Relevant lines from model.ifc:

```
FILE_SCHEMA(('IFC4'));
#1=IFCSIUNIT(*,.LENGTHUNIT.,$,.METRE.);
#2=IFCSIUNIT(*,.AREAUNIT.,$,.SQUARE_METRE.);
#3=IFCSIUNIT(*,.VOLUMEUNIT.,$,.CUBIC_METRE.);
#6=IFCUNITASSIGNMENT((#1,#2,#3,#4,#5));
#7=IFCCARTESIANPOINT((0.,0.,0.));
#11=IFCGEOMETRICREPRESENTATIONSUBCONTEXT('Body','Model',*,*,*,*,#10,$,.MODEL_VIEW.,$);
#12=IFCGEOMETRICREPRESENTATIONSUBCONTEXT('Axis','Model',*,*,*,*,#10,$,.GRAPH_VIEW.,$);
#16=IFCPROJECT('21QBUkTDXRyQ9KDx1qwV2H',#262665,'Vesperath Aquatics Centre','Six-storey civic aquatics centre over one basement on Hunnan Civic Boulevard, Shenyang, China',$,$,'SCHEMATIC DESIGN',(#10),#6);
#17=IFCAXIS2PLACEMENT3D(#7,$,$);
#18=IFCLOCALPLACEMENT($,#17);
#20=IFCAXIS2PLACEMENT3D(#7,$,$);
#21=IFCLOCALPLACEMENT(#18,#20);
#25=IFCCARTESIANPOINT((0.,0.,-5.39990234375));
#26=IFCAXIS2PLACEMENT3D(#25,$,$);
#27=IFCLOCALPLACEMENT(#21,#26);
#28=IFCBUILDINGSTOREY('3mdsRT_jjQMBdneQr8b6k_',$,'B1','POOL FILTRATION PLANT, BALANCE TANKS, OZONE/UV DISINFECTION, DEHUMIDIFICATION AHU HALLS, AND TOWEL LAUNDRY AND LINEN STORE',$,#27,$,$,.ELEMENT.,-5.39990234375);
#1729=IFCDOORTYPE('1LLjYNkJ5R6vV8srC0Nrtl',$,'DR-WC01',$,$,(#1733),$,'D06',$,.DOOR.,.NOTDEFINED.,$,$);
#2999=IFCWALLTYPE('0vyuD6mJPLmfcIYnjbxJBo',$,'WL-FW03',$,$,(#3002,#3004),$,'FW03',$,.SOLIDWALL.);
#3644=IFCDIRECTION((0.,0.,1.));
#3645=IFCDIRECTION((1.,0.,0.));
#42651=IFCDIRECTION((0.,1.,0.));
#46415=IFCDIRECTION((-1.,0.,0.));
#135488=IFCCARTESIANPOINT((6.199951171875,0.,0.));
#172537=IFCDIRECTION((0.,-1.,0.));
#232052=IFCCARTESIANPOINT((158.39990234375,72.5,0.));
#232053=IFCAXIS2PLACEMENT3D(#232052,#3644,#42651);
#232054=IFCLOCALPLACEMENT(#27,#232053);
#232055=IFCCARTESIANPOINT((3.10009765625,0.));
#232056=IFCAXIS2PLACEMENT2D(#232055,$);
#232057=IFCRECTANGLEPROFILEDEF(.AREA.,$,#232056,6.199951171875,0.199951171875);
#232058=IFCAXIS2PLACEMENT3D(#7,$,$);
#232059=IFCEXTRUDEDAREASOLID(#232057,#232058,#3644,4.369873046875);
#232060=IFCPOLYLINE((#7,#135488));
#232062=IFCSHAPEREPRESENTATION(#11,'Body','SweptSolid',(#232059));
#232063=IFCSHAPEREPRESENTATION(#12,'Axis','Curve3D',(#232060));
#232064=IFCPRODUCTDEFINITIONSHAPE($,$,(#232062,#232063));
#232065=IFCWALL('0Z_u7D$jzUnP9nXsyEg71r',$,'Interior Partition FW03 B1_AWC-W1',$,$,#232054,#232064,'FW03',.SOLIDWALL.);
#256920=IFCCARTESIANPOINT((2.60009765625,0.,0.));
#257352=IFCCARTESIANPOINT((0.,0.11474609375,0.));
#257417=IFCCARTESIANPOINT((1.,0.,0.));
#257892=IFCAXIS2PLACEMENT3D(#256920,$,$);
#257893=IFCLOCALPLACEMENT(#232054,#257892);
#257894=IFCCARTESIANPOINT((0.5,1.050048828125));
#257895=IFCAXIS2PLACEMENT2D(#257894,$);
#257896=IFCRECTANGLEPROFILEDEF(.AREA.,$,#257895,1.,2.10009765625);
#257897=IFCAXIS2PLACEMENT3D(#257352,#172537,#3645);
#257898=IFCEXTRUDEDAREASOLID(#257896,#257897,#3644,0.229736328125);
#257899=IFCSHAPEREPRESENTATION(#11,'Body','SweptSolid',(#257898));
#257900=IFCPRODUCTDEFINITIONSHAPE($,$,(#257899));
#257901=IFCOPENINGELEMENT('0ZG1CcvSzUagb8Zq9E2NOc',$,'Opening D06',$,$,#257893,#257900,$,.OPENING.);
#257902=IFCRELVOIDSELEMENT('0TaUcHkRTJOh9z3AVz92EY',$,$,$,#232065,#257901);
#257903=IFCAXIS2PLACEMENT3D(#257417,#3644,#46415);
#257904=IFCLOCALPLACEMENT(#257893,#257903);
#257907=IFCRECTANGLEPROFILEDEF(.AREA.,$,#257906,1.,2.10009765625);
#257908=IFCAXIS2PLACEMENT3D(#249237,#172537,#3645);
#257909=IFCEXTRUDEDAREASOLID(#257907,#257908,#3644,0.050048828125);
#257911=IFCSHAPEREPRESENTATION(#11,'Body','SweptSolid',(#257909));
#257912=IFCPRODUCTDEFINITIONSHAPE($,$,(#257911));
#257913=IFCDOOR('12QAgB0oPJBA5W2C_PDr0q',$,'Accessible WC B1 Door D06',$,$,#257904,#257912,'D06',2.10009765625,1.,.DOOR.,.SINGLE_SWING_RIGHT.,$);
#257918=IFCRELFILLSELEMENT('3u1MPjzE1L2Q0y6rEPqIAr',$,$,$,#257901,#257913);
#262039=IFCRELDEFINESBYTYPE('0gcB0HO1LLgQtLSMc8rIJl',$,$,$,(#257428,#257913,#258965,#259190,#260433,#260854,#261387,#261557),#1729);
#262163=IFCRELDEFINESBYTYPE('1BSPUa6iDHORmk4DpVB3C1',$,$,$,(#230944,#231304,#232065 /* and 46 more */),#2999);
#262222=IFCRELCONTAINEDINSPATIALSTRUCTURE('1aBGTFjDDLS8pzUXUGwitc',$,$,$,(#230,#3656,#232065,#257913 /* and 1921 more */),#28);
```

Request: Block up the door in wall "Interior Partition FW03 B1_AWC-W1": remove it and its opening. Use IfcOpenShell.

```python
import ifcopenshell
import ifcopenshell.api.feature
import ifcopenshell.api.root
import ifcopenshell.geom
import ifcopenshell.util.shape

model = ifcopenshell.open("model.ifc")
settings = ifcopenshell.geom.settings()


def volume(element):
    """Net volume in cubic metres, openings subtracted."""
    shape = ifcopenshell.geom.create_shape(settings, element)
    return ifcopenshell.util.shape.get_volume(shape.geometry)


door = model.by_guid("12QAgB0oPJBA5W2C_PDr0q")
opening = door.FillsVoids[0].RelatingOpeningElement
wall = opening.VoidsElements[0].RelatingBuildingElement
before = volume(wall)

ifcopenshell.api.root.remove_product(model, product=door)
ifcopenshell.api.feature.remove_feature(model, feature=opening)

after = volume(wall)

print(f"wall volume {before:.3f} -> {after:.3f} m3")

model.write("model_edited.ifc")
```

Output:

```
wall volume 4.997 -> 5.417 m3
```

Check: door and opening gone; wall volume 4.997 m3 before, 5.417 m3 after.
